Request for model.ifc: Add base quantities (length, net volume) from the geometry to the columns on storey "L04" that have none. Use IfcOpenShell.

First a look at what the model holds.

```python
import ifcopenshell
import ifcopenshell.util.element
import ifcopenshell.util.unit

model = ifcopenshell.open("model.ifc")
print(model.schema)
for unit_type in ("LENGTHUNIT", "AREAUNIT", "VOLUMEUNIT"):
    print(unit_type, ifcopenshell.util.unit.calculate_unit_scale(model, unit_type))
storey = next(s for s in model.by_type("IfcBuildingStorey") if s.Name == "L04")
columns = [e for e in ifcopenshell.util.element.get_decomposition(storey) if e.is_a("IfcColumn")]
for e in sorted(columns, key=lambda e: e.id()):
    print(e.id(), e.is_a(), e.Name, list(ifcopenshell.util.element.get_psets(e, qtos_only=True)), sep=" | ")
```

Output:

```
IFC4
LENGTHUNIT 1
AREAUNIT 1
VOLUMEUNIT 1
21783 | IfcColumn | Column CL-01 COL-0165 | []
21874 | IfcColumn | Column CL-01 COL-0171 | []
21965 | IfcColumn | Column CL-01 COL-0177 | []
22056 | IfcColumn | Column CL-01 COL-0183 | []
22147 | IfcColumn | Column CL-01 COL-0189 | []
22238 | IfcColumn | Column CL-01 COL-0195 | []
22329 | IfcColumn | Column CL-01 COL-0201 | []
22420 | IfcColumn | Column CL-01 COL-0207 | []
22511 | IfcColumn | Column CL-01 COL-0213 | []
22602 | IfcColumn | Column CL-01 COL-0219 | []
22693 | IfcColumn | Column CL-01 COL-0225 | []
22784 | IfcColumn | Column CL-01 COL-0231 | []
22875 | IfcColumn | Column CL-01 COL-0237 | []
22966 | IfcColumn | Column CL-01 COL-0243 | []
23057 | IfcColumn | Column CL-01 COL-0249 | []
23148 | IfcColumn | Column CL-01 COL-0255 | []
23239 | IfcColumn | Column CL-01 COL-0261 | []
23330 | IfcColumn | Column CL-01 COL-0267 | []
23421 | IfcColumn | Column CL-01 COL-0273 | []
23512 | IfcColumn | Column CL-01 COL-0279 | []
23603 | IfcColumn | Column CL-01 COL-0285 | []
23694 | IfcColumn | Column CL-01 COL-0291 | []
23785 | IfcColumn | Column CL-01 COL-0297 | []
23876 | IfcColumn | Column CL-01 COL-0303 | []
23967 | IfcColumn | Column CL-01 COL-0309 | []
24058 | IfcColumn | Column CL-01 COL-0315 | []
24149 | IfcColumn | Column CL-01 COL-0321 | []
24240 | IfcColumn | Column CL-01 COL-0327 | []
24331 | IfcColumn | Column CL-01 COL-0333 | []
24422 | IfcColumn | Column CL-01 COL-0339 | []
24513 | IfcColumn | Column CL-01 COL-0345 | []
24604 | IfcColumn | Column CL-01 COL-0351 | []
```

```python
import ifcopenshell
import ifcopenshell.api.pset
import ifcopenshell.geom
import ifcopenshell.util.element
import ifcopenshell.util.shape
import ifcopenshell.util.unit

model = ifcopenshell.open("model.ifc")
unit_scale = ifcopenshell.util.unit.calculate_unit_scale(model)
volume_scale = ifcopenshell.util.unit.calculate_unit_scale(model, "VOLUMEUNIT")
settings = ifcopenshell.geom.settings()

storey = next(s for s in model.by_type("IfcBuildingStorey") if s.Name == "L04")
columns = [e for e in ifcopenshell.util.element.get_decomposition(storey) if e.is_a("IfcColumn")]

for e in sorted(columns, key=lambda e: e.id()):
    if ifcopenshell.util.element.get_psets(e, qtos_only=True, should_inherit=False):
        continue
    # Geometry comes back in metres, in the element's own axes.
    shape = ifcopenshell.geom.create_shape(settings, e)
    values = {
        "Length": ifcopenshell.util.shape.get_z(shape.geometry) / unit_scale,
        "NetVolume": ifcopenshell.util.shape.get_volume(shape.geometry) / volume_scale,
    }
    qto = ifcopenshell.api.pset.add_qto(model, product=e, name="Qto_ColumnBaseQuantities")
    ifcopenshell.api.pset.edit_qto(model, qto=qto, properties=values)
    print(e.id(), {k: round(v, 3) for k, v in values.items()})

model.write("model_rev.ifc")
```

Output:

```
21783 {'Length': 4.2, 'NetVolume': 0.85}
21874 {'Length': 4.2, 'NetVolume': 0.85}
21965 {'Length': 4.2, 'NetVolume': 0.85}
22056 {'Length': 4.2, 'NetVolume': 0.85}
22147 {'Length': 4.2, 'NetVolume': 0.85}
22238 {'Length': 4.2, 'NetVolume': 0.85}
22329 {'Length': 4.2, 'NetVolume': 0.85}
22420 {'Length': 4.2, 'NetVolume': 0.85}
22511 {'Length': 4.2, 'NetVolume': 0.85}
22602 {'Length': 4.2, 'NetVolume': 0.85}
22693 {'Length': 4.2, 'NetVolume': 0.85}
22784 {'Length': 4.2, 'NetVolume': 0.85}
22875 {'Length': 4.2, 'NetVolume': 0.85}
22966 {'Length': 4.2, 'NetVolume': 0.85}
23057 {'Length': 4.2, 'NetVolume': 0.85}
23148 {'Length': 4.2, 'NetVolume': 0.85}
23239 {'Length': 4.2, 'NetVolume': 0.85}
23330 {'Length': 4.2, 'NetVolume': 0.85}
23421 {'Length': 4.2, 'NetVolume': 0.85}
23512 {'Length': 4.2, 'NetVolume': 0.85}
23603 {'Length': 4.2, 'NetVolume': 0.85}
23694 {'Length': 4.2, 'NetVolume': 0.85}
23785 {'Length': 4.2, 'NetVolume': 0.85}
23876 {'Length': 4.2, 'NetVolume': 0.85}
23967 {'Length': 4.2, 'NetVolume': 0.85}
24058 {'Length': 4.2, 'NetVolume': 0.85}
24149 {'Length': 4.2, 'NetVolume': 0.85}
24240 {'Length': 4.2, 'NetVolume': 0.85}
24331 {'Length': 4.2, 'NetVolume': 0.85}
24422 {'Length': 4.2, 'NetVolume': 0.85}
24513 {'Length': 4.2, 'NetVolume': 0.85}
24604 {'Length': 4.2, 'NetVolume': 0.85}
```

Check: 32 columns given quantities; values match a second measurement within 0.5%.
